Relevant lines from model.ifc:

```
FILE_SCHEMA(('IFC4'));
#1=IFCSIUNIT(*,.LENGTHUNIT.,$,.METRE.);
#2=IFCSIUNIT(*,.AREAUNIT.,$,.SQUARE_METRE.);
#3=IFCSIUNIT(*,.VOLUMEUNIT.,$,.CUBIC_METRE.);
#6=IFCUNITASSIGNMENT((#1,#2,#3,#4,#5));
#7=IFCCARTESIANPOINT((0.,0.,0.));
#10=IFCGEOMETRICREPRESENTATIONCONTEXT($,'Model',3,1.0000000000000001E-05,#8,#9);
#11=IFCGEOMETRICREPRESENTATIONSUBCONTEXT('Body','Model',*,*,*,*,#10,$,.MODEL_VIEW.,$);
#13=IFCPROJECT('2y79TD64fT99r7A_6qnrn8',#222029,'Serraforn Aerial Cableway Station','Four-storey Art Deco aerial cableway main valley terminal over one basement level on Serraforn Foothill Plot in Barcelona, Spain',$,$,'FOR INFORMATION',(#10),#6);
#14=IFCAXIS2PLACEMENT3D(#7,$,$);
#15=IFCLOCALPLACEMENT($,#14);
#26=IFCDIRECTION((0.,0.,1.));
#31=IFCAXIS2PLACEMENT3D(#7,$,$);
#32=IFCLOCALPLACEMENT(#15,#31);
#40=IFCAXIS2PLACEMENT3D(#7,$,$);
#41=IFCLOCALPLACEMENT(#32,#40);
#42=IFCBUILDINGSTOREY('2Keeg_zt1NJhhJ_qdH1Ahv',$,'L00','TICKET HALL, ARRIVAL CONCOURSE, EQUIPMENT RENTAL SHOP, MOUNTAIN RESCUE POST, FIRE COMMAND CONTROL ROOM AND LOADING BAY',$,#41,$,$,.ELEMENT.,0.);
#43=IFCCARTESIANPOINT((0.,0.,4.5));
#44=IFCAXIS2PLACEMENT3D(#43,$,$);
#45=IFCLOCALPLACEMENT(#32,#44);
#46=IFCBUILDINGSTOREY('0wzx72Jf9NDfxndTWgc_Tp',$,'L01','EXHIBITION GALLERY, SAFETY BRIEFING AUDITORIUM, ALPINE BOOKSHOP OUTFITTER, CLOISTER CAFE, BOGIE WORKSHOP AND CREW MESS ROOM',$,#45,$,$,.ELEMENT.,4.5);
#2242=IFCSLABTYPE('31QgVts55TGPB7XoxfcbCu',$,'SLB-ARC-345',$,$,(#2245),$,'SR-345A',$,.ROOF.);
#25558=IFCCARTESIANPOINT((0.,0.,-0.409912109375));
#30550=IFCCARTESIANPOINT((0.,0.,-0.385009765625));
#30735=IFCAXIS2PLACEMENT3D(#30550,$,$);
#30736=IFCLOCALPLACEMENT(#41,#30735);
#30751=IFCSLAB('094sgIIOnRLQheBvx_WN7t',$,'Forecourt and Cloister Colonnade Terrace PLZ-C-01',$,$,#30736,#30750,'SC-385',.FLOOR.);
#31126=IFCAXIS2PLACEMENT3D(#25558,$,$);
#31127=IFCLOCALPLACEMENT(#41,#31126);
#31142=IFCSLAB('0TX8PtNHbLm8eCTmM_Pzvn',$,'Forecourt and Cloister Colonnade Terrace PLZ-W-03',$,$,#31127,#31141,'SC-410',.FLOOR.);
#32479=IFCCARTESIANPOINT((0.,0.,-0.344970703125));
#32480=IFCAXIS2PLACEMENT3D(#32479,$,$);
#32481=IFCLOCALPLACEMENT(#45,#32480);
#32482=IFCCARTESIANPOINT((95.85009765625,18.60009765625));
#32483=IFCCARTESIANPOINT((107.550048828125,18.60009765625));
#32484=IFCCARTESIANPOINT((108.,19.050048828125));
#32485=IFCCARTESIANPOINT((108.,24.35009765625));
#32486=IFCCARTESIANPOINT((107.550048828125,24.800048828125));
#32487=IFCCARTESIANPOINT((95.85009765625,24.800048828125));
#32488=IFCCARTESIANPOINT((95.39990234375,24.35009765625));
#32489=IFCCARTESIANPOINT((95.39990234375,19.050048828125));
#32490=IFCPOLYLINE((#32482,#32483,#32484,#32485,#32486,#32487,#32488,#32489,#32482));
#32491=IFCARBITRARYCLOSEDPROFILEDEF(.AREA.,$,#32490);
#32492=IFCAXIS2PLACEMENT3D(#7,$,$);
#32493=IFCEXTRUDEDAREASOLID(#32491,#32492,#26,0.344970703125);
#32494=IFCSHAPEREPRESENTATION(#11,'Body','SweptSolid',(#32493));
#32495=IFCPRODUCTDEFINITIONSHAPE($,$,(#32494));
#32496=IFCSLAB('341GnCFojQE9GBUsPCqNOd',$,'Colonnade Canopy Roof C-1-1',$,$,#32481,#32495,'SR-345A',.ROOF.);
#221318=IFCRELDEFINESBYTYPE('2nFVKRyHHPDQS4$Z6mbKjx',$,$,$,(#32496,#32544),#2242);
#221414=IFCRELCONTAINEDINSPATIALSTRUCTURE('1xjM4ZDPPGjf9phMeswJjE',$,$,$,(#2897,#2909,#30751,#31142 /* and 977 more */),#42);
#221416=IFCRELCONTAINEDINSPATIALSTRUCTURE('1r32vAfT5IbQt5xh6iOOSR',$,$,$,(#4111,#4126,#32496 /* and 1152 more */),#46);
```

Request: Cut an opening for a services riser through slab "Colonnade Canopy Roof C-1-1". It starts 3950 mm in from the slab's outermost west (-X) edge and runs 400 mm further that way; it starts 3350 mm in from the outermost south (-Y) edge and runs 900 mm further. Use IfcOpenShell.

```python
import numpy as np
import ifcopenshell
import ifcopenshell.api.feature
import ifcopenshell.api.geometry
import ifcopenshell.api.root
import ifcopenshell.geom
import ifcopenshell.util.placement
import ifcopenshell.util.representation
import ifcopenshell.util.shape
import ifcopenshell.util.unit

model = ifcopenshell.open("model.ifc")
unit_scale = ifcopenshell.util.unit.calculate_unit_scale(model)
settings = ifcopenshell.geom.settings()


def volume(element):
    """Net volume in cubic metres, openings subtracted."""
    shape = ifcopenshell.geom.create_shape(settings, element)
    return ifcopenshell.util.shape.get_volume(shape.geometry)


slab = model.by_guid("341GnCFojQE9GBUsPCqNOd")
before = volume(slab)

# Extent in the slab's own axes, in metres. The edges named are its -X and -Y sides.
slab_shape = ifcopenshell.geom.create_shape(settings, slab)
vertices = ifcopenshell.util.shape.get_vertices(slab_shape.geometry)
x_min, y_min, bottom = vertices.min(axis=0)
top = vertices[:, 2].max()

opening = ifcopenshell.api.root.create_entity(model, ifc_class="IfcOpeningElement", name="Services riser opening", predefined_type="OPENING")
context = ifcopenshell.util.representation.get_context(model, "Model", "Body", "MODEL_VIEW")
width, depth = 0.4, 0.9
outline = [(0.0, 0.0), (width, 0.0), (width, depth), (0.0, depth), (0.0, 0.0)]
# Overshoot both faces by 50 mm so the cut is clean.
shape = ifcopenshell.api.geometry.add_slab_representation(
    model, context=context, depth=top - bottom + 0.1, polyline=outline
)
ifcopenshell.api.geometry.assign_representation(model, product=opening, representation=shape)

matrix = ifcopenshell.util.placement.get_local_placement(slab.ObjectPlacement)
matrix[:, 3] = matrix @ np.append(np.array([x_min + 3.95, y_min + 3.35, bottom - 0.05]) / unit_scale, 1.0)
ifcopenshell.api.geometry.edit_object_placement(model, product=opening, matrix=matrix, is_si=False)
ifcopenshell.api.feature.add_feature(model, feature=opening, element=slab)

after = volume(slab)

print(f"slab volume {before:.3f} -> {after:.3f} m3")

model.write("model_updated.ifc")
```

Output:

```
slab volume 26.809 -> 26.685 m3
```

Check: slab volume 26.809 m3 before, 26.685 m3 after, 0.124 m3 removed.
